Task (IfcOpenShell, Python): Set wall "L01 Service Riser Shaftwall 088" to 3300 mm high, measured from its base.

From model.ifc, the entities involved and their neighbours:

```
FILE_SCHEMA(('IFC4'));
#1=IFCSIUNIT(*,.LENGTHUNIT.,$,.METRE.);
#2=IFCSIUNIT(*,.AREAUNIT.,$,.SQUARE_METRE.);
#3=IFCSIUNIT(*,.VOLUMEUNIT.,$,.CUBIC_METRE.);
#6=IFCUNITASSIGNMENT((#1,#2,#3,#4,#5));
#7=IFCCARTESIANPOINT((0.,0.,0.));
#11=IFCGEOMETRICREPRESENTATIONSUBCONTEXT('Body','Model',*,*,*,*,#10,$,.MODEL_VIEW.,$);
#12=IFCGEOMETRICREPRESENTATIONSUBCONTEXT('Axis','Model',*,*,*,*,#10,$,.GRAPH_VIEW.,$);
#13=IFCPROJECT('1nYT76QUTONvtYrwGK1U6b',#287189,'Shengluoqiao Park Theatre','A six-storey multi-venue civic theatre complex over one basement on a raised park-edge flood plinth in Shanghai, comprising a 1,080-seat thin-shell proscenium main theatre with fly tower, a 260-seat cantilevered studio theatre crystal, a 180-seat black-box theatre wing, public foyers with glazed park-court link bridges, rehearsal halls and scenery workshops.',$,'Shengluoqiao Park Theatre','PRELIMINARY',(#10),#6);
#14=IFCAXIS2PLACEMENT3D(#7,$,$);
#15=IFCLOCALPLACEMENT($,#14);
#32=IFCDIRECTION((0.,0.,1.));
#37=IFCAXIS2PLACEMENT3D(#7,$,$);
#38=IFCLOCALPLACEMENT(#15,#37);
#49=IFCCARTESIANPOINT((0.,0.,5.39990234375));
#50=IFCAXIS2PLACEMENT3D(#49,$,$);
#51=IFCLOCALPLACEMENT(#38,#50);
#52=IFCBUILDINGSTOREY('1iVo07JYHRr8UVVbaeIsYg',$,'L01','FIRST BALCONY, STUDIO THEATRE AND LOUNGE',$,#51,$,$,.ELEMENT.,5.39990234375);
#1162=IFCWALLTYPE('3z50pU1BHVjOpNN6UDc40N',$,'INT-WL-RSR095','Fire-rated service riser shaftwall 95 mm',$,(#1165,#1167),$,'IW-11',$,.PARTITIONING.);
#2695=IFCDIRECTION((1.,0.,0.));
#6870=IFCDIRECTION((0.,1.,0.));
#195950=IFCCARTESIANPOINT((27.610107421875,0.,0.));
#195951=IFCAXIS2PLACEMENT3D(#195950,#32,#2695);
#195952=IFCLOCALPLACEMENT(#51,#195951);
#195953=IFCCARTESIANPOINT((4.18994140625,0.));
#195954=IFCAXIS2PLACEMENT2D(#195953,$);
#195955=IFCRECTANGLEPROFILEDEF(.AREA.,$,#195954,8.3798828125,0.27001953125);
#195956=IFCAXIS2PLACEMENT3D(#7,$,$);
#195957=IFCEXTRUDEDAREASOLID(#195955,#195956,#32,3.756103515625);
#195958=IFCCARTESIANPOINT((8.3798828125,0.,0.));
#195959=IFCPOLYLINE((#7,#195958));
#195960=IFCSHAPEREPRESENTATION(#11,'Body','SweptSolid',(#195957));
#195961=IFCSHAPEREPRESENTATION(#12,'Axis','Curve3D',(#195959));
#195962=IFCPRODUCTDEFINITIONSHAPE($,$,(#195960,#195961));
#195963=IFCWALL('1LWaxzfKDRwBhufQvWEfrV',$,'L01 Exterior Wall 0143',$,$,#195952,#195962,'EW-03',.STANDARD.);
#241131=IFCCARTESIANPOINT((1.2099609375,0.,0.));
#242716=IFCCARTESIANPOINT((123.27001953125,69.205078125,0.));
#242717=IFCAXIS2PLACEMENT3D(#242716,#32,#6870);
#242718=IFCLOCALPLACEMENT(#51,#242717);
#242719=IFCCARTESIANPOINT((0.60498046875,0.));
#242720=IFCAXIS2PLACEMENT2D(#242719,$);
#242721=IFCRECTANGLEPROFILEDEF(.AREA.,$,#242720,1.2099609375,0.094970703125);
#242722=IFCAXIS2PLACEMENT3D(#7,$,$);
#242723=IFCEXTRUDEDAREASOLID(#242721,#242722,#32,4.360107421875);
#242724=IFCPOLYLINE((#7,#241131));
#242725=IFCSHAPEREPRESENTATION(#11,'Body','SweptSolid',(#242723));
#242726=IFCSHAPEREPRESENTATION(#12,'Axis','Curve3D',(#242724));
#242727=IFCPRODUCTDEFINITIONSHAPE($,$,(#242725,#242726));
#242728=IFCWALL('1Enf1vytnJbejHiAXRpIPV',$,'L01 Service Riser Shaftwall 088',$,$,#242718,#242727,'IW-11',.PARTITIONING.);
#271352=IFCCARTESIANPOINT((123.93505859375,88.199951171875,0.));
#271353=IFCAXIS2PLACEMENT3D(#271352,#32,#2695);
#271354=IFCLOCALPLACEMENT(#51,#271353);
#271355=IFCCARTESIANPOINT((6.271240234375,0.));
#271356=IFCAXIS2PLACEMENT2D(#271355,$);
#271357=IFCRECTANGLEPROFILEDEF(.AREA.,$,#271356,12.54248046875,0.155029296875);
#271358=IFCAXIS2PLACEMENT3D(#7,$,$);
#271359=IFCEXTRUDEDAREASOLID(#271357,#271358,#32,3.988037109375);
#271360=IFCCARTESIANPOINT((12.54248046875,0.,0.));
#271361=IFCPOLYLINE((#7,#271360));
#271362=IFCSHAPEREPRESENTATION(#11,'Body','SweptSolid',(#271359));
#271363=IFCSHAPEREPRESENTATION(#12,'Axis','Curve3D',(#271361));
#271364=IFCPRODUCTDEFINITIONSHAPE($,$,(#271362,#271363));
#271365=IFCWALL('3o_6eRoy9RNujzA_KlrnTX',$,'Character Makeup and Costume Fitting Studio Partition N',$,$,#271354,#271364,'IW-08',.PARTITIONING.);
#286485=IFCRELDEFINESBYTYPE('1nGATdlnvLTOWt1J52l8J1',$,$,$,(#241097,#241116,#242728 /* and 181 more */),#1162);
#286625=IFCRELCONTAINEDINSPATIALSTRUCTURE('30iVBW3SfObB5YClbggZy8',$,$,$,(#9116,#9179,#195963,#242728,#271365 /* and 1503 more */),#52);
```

```python
import ifcopenshell
import ifcopenshell.geom
import ifcopenshell.util.representation
import ifcopenshell.util.shape
import ifcopenshell.util.unit

model = ifcopenshell.open("model.ifc")
unit_scale = ifcopenshell.util.unit.calculate_unit_scale(model)
settings = ifcopenshell.geom.settings()


def volume(element):
    """Net volume in cubic metres, openings subtracted."""
    shape = ifcopenshell.geom.create_shape(settings, element)
    return ifcopenshell.util.shape.get_volume(shape.geometry)


wall = model.by_guid("1Enf1vytnJbejHiAXRpIPV")
before = volume(wall)

body = ifcopenshell.util.representation.get_representation(wall, "Model", "Body")
solid = body.Items[0]
old_height = solid.Depth
solid.Depth = 3.3 / unit_scale
after = volume(wall)

print(f"height {old_height:g} -> {solid.Depth:g}, volume {before:.3f} -> {after:.3f} m3")

model.write("model-out.ifc")
```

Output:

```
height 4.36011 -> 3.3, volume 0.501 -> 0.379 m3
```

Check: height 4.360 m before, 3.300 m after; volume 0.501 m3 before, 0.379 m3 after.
